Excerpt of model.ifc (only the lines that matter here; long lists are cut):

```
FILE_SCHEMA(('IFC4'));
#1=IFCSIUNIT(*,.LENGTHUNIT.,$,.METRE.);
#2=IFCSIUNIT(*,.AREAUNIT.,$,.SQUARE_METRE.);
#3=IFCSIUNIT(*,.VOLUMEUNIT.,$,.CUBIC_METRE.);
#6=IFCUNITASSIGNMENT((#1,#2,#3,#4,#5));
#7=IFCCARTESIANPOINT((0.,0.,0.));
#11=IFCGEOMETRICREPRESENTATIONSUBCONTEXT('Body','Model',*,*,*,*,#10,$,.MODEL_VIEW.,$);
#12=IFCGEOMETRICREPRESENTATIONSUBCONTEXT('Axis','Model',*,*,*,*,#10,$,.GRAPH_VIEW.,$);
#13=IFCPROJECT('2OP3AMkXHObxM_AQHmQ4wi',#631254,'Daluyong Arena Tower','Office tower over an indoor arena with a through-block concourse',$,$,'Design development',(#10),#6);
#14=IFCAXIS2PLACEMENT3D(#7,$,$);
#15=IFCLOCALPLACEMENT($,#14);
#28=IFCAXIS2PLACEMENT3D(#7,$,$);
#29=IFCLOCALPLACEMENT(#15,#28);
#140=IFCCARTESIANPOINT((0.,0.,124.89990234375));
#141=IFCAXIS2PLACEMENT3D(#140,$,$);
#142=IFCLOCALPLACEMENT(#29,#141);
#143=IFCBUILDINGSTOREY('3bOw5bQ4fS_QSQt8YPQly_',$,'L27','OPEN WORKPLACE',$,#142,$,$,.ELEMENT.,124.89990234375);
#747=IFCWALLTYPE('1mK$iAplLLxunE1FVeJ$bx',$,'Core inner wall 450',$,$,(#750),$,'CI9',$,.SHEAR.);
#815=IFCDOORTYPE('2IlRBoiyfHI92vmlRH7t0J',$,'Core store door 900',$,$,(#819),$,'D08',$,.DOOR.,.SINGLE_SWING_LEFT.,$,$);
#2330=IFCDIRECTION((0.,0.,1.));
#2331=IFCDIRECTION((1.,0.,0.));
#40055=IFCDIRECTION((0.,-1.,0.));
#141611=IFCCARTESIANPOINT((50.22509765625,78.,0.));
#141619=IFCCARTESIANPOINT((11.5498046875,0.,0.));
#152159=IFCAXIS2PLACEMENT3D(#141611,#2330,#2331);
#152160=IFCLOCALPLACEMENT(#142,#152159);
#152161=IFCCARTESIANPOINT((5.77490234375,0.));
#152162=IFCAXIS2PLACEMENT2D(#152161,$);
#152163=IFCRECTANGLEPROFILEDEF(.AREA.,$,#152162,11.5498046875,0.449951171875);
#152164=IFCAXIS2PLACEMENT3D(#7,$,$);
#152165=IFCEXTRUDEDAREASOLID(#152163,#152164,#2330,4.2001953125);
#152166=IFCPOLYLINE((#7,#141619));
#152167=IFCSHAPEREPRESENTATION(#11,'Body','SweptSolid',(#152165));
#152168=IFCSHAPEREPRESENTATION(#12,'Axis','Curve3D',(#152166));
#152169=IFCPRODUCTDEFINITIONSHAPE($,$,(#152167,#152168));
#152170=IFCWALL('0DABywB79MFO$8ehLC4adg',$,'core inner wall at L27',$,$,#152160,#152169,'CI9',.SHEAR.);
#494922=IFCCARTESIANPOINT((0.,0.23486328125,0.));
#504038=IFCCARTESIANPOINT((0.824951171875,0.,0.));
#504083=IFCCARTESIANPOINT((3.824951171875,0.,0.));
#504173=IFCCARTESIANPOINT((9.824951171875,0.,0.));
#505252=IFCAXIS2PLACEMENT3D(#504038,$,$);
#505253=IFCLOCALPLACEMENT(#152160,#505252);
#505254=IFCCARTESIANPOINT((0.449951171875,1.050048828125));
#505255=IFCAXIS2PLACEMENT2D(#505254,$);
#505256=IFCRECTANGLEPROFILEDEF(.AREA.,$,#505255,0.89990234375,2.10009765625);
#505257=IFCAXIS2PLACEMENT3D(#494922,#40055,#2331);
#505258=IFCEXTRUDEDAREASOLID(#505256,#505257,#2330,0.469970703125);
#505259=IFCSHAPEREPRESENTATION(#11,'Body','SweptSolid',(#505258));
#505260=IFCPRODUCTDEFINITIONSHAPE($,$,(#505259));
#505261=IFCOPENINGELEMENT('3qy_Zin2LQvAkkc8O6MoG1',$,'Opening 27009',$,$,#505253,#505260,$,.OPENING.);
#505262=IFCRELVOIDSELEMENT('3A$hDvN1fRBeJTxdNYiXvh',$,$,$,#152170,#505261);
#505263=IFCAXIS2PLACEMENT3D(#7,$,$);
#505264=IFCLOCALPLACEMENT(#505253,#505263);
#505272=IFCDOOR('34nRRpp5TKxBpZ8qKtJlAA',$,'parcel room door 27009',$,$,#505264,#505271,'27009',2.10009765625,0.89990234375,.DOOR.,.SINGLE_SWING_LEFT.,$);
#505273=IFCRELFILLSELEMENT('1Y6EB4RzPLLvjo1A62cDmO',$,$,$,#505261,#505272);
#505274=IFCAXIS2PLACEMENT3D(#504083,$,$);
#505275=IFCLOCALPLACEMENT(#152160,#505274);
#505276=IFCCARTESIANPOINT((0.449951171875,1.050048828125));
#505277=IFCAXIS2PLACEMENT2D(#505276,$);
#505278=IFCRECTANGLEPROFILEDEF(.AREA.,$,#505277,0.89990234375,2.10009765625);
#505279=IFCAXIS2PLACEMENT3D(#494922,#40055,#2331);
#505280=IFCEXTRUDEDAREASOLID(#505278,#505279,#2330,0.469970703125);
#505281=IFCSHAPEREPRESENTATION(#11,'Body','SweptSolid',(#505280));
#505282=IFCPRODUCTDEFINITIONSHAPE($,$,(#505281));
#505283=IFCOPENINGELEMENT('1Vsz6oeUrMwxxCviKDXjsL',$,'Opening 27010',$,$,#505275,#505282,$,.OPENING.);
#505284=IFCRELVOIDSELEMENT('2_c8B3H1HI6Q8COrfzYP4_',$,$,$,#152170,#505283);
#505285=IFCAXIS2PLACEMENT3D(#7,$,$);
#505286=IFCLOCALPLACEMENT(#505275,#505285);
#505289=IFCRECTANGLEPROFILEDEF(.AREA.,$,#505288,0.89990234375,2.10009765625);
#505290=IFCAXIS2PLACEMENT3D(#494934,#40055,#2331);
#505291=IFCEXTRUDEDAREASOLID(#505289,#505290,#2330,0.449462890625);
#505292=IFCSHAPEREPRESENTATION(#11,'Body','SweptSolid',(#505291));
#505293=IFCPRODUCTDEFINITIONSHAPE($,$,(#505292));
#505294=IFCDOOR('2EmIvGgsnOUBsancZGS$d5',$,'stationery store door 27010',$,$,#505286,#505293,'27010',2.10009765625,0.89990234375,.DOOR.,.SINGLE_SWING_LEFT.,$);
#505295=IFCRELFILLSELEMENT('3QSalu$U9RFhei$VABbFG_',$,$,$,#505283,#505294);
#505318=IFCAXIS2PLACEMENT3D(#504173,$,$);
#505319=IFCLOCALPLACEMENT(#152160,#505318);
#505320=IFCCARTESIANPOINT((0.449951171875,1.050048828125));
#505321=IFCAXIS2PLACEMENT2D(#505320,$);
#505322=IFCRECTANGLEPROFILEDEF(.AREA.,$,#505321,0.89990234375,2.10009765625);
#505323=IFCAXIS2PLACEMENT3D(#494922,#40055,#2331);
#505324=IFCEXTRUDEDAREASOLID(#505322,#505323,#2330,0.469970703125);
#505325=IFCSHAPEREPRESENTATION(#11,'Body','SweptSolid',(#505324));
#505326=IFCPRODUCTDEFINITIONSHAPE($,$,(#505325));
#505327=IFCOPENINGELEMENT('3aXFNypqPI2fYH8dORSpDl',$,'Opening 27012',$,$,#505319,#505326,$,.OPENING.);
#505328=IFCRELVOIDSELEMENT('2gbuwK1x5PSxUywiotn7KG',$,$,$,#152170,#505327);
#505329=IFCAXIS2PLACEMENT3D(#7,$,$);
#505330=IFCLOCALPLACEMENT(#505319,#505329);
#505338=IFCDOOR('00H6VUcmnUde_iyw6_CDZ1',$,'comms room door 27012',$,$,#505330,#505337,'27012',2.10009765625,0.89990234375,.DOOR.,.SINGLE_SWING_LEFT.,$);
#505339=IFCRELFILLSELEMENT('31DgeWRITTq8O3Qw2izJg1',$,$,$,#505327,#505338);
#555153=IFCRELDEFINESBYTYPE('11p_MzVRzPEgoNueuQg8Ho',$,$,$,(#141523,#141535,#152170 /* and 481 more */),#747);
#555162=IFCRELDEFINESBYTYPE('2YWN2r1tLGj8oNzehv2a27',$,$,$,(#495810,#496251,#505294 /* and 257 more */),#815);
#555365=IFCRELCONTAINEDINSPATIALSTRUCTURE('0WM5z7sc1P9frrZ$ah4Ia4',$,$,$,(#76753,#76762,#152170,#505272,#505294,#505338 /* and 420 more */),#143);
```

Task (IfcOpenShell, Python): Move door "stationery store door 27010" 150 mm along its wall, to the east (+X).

```python
import ifcopenshell
import ifcopenshell.api.geometry
import ifcopenshell.util.placement

model = ifcopenshell.open("model.ifc")

door = model.by_guid("2EmIvGgsnOUBsancZGS$d5")
opening = door.FillsVoids[0].RelatingOpeningElement
wall = opening.VoidsElements[0].RelatingBuildingElement

wall_matrix = ifcopenshell.util.placement.get_local_placement(wall.ObjectPlacement)
shift = wall_matrix[:3, 0] * 0.15
before = ifcopenshell.util.placement.get_local_placement(door.ObjectPlacement)[:3, 3].copy()

# The door is placed relative to its opening, so it follows when the opening moves.
matrix = ifcopenshell.util.placement.get_local_placement(opening.ObjectPlacement)
matrix[:3, 3] += shift
ifcopenshell.api.geometry.edit_object_placement(
    model, product=opening, matrix=matrix, is_si=False, should_transform_children=True
)

after = ifcopenshell.util.placement.get_local_placement(door.ObjectPlacement)[:3, 3]
print("door moved by", (after - before).round(3) + 0.0)

model.write("model_v2.ifc")
```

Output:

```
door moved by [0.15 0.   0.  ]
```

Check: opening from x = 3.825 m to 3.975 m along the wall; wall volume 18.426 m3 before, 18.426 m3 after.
